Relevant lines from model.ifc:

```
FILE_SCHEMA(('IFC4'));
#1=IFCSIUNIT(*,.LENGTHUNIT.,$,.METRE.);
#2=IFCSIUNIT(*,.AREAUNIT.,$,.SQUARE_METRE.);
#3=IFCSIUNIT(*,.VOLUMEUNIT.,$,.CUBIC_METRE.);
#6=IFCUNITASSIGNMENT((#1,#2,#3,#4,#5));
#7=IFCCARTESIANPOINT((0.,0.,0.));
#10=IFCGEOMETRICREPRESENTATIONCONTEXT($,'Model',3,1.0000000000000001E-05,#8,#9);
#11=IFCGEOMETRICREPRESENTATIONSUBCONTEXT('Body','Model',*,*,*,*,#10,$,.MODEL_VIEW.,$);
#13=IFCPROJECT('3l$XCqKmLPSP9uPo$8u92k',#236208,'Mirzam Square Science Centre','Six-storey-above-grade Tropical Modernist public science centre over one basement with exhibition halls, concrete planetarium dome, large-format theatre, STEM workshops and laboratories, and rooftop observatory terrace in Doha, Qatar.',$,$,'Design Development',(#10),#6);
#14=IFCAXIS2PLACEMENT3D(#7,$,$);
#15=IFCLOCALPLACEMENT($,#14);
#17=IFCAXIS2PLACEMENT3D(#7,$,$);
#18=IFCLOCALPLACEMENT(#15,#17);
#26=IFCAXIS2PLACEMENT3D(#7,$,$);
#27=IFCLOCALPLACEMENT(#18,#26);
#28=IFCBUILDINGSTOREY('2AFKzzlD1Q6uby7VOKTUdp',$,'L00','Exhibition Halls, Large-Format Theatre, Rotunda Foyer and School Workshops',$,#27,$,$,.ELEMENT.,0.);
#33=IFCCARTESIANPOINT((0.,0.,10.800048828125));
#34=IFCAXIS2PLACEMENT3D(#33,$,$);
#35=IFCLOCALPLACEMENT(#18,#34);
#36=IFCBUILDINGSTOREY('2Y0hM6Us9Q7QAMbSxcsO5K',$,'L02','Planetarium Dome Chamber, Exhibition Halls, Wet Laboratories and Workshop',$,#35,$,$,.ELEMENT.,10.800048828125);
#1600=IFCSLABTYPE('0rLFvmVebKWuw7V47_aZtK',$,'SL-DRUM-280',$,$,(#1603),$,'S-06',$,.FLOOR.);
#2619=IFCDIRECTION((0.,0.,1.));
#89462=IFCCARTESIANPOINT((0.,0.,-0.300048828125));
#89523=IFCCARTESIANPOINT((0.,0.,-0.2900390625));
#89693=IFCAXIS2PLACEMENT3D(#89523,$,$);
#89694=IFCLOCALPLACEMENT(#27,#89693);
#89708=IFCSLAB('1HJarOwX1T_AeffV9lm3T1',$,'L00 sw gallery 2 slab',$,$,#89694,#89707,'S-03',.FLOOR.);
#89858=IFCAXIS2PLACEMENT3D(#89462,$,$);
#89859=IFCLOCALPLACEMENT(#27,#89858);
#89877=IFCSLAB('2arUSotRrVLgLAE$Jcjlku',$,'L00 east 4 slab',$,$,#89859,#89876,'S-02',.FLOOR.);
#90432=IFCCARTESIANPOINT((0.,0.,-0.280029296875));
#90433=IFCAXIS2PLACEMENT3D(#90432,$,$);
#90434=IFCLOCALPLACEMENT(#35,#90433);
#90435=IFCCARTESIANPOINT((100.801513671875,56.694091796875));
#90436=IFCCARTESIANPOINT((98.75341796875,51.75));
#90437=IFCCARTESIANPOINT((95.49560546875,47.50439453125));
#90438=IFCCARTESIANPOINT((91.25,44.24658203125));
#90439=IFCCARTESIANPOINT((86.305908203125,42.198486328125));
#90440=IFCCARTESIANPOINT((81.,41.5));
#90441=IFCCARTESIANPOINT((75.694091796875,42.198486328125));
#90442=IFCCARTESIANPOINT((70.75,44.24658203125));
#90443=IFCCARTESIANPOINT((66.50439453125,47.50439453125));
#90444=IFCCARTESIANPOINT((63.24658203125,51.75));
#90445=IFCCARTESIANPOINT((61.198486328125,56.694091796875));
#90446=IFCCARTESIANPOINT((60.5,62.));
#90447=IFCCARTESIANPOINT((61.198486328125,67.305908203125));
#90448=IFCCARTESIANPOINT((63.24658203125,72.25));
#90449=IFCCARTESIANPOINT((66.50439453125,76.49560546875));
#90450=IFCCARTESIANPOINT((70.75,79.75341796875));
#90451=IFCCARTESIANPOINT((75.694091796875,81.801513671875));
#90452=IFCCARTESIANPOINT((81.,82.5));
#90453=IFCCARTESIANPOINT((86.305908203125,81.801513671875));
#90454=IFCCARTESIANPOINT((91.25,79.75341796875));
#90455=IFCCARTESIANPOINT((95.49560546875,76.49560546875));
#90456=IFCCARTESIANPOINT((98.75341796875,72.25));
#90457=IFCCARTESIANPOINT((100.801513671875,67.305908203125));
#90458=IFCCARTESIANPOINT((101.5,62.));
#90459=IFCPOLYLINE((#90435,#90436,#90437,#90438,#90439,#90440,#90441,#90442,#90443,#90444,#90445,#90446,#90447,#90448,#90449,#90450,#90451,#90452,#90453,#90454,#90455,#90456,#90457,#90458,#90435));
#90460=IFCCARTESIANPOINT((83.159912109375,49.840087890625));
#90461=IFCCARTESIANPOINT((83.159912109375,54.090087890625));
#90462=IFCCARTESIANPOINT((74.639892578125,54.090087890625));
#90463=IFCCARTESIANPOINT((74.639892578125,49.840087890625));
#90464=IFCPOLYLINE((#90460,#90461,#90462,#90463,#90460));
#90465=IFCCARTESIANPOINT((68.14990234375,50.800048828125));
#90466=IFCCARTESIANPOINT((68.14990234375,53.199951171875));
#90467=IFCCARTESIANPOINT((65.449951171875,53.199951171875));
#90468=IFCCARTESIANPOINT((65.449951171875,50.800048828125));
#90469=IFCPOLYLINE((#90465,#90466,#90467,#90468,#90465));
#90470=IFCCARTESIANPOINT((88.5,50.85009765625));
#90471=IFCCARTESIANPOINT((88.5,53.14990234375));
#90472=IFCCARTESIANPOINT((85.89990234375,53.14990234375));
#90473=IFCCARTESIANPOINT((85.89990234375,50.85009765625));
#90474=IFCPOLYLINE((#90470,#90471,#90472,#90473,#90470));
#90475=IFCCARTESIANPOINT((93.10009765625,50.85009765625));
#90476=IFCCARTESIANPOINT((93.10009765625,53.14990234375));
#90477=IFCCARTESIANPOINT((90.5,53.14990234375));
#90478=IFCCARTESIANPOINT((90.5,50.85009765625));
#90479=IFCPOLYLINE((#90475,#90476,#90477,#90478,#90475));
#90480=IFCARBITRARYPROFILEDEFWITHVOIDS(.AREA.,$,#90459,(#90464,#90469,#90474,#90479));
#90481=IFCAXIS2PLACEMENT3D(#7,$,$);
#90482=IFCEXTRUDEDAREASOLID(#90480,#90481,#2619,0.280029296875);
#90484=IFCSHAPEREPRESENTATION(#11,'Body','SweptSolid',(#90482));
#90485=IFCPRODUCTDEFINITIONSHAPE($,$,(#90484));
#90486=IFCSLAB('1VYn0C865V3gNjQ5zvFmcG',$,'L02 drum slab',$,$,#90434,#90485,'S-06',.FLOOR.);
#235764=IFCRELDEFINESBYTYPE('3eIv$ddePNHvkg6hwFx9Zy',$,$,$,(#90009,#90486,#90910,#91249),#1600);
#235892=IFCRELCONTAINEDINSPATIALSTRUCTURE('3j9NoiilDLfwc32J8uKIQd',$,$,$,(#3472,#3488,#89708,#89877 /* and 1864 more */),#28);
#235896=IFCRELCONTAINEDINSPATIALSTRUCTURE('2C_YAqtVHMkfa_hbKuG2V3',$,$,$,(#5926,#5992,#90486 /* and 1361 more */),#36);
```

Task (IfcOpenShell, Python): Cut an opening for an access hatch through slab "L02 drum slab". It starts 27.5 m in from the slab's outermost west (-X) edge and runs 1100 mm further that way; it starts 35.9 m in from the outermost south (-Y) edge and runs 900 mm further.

```python
import numpy as np
import ifcopenshell
import ifcopenshell.api.feature
import ifcopenshell.api.geometry
import ifcopenshell.api.root
import ifcopenshell.geom
import ifcopenshell.util.placement
import ifcopenshell.util.representation
import ifcopenshell.util.shape
import ifcopenshell.util.unit

model = ifcopenshell.open("model.ifc")
unit_scale = ifcopenshell.util.unit.calculate_unit_scale(model)
settings = ifcopenshell.geom.settings()


def volume(element):
    """Net volume in cubic metres, openings subtracted."""
    shape = ifcopenshell.geom.create_shape(settings, element)
    return ifcopenshell.util.shape.get_volume(shape.geometry)


slab = model.by_guid("1VYn0C865V3gNjQ5zvFmcG")
before = volume(slab)

# Extent in the slab's own axes, in metres. The edges named are its -X and -Y sides.
slab_shape = ifcopenshell.geom.create_shape(settings, slab)
vertices = ifcopenshell.util.shape.get_vertices(slab_shape.geometry)
x_min, y_min, bottom = vertices.min(axis=0)
top = vertices[:, 2].max()

opening = ifcopenshell.api.root.create_entity(model, ifc_class="IfcOpeningElement", name="Access hatch opening", predefined_type="OPENING")
context = ifcopenshell.util.representation.get_context(model, "Model", "Body", "MODEL_VIEW")
width, depth = 1.1, 0.9
outline = [(0.0, 0.0), (width, 0.0), (width, depth), (0.0, depth), (0.0, 0.0)]
# Overshoot both faces by 50 mm so the cut is clean.
shape = ifcopenshell.api.geometry.add_slab_representation(
    model, context=context, depth=top - bottom + 0.1, polyline=outline
)
ifcopenshell.api.geometry.assign_representation(model, product=opening, representation=shape)

matrix = ifcopenshell.util.placement.get_local_placement(slab.ObjectPlacement)
matrix[:, 3] = matrix @ np.append(np.array([x_min + 27.5, y_min + 35.9, bottom - 0.05]) / unit_scale, 1.0)
ifcopenshell.api.geometry.edit_object_placement(model, product=opening, matrix=matrix, is_si=False)
ifcopenshell.api.feature.add_feature(model, feature=opening, element=slab)

after = volume(slab)

print(f"slab volume {before:.3f} -> {after:.3f} m3")

model.write("model-out.ifc")
```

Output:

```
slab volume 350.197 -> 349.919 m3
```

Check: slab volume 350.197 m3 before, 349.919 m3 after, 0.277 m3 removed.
